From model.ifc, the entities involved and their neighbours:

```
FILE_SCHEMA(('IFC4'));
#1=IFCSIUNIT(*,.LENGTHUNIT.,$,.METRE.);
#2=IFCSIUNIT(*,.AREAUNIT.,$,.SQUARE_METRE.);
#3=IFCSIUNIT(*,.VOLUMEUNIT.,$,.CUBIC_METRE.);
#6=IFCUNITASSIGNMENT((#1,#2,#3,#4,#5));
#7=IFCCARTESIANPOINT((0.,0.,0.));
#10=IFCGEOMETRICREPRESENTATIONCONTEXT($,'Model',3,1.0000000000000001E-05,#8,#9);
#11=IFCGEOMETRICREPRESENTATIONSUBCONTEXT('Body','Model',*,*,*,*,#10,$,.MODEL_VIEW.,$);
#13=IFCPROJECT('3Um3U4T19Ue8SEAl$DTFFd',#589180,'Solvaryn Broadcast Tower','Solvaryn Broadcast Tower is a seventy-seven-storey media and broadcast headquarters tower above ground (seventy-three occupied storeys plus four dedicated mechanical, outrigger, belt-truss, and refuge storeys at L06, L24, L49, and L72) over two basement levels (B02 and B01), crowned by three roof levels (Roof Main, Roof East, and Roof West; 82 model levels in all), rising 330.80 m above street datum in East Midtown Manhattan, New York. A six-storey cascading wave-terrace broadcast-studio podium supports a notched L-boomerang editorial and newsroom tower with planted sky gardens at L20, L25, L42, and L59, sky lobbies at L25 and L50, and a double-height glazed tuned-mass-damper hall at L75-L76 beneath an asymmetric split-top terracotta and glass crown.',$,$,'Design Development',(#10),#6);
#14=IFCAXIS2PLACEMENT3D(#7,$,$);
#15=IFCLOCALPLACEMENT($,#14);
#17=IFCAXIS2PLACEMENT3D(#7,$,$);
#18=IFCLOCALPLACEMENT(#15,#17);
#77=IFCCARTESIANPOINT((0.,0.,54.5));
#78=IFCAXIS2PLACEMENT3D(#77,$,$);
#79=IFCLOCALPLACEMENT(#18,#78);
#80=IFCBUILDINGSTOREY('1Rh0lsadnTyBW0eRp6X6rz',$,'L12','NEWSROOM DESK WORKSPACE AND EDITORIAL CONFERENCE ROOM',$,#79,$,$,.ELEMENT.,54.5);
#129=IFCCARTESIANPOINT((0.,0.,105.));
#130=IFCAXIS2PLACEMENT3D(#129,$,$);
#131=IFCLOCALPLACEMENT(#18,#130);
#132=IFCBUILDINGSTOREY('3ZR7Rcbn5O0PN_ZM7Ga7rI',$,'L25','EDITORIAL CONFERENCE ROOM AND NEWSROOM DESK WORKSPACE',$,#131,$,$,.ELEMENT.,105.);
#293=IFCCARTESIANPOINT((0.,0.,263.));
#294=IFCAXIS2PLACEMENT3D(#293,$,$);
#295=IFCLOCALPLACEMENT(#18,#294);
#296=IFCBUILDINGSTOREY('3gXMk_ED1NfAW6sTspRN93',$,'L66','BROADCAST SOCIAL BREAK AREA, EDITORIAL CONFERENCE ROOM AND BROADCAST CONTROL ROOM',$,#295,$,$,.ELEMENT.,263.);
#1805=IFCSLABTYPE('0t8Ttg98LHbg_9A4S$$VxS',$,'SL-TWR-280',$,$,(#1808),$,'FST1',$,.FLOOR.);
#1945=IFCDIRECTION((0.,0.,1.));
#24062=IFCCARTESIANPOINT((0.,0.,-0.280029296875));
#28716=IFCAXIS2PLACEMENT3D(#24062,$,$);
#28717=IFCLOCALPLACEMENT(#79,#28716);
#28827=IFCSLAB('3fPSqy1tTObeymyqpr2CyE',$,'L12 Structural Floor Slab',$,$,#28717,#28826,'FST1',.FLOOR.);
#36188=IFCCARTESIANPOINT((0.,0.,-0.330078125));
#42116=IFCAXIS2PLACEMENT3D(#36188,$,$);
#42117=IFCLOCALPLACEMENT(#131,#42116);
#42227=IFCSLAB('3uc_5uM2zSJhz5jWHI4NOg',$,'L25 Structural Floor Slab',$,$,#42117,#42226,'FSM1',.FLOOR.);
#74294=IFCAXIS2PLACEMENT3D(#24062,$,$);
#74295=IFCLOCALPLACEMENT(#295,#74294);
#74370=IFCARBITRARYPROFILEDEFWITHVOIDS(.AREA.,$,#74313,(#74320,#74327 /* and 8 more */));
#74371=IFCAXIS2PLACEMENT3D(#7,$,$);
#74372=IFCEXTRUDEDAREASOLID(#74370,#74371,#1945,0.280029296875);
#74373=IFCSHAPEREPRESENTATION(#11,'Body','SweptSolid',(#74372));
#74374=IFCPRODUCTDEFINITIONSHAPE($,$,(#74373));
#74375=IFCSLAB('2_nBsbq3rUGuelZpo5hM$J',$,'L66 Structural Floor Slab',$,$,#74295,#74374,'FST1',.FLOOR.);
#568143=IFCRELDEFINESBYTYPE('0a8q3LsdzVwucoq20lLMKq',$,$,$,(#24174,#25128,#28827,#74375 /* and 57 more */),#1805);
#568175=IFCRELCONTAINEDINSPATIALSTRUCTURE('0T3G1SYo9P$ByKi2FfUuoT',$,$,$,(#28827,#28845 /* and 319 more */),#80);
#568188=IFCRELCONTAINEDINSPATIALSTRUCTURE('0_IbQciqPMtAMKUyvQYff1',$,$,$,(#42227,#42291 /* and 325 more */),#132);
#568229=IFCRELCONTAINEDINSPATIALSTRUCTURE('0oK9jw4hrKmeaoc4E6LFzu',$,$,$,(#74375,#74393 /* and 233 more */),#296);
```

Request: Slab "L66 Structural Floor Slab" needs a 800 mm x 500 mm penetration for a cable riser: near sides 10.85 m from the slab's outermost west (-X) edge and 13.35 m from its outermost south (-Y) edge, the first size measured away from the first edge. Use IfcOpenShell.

```python
import numpy as np
import ifcopenshell
import ifcopenshell.api.feature
import ifcopenshell.api.geometry
import ifcopenshell.api.root
import ifcopenshell.geom
import ifcopenshell.util.placement
import ifcopenshell.util.representation
import ifcopenshell.util.shape
import ifcopenshell.util.unit

model = ifcopenshell.open("model.ifc")
unit_scale = ifcopenshell.util.unit.calculate_unit_scale(model)
settings = ifcopenshell.geom.settings()


def volume(element):
    """Net volume in cubic metres, openings subtracted."""
    shape = ifcopenshell.geom.create_shape(settings, element)
    return ifcopenshell.util.shape.get_volume(shape.geometry)


slab = model.by_guid("2_nBsbq3rUGuelZpo5hM$J")
before = volume(slab)

# Extent in the slab's own axes, in metres. The edges named are its -X and -Y sides.
slab_shape = ifcopenshell.geom.create_shape(settings, slab)
vertices = ifcopenshell.util.shape.get_vertices(slab_shape.geometry)
x_min, y_min, bottom = vertices.min(axis=0)
top = vertices[:, 2].max()

opening = ifcopenshell.api.root.create_entity(model, ifc_class="IfcOpeningElement", name="Cable riser opening", predefined_type="OPENING")
context = ifcopenshell.util.representation.get_context(model, "Model", "Body", "MODEL_VIEW")
width, depth = 0.8, 0.5
outline = [(0.0, 0.0), (width, 0.0), (width, depth), (0.0, depth), (0.0, 0.0)]
# Overshoot both faces by 50 mm so the cut is clean.
shape = ifcopenshell.api.geometry.add_slab_representation(
    model, context=context, depth=top - bottom + 0.1, polyline=outline
)
ifcopenshell.api.geometry.assign_representation(model, product=opening, representation=shape)

matrix = ifcopenshell.util.placement.get_local_placement(slab.ObjectPlacement)
matrix[:, 3] = matrix @ np.append(np.array([x_min + 10.85, y_min + 13.35, bottom - 0.05]) / unit_scale, 1.0)
ifcopenshell.api.geometry.edit_object_placement(model, product=opening, matrix=matrix, is_si=False)
ifcopenshell.api.feature.add_feature(model, feature=opening, element=slab)

after = volume(slab)

print(f"slab volume {before:.3f} -> {after:.3f} m3")

model.write("model_rev.ifc")
```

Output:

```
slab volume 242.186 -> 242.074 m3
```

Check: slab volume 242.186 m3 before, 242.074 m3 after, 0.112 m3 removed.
